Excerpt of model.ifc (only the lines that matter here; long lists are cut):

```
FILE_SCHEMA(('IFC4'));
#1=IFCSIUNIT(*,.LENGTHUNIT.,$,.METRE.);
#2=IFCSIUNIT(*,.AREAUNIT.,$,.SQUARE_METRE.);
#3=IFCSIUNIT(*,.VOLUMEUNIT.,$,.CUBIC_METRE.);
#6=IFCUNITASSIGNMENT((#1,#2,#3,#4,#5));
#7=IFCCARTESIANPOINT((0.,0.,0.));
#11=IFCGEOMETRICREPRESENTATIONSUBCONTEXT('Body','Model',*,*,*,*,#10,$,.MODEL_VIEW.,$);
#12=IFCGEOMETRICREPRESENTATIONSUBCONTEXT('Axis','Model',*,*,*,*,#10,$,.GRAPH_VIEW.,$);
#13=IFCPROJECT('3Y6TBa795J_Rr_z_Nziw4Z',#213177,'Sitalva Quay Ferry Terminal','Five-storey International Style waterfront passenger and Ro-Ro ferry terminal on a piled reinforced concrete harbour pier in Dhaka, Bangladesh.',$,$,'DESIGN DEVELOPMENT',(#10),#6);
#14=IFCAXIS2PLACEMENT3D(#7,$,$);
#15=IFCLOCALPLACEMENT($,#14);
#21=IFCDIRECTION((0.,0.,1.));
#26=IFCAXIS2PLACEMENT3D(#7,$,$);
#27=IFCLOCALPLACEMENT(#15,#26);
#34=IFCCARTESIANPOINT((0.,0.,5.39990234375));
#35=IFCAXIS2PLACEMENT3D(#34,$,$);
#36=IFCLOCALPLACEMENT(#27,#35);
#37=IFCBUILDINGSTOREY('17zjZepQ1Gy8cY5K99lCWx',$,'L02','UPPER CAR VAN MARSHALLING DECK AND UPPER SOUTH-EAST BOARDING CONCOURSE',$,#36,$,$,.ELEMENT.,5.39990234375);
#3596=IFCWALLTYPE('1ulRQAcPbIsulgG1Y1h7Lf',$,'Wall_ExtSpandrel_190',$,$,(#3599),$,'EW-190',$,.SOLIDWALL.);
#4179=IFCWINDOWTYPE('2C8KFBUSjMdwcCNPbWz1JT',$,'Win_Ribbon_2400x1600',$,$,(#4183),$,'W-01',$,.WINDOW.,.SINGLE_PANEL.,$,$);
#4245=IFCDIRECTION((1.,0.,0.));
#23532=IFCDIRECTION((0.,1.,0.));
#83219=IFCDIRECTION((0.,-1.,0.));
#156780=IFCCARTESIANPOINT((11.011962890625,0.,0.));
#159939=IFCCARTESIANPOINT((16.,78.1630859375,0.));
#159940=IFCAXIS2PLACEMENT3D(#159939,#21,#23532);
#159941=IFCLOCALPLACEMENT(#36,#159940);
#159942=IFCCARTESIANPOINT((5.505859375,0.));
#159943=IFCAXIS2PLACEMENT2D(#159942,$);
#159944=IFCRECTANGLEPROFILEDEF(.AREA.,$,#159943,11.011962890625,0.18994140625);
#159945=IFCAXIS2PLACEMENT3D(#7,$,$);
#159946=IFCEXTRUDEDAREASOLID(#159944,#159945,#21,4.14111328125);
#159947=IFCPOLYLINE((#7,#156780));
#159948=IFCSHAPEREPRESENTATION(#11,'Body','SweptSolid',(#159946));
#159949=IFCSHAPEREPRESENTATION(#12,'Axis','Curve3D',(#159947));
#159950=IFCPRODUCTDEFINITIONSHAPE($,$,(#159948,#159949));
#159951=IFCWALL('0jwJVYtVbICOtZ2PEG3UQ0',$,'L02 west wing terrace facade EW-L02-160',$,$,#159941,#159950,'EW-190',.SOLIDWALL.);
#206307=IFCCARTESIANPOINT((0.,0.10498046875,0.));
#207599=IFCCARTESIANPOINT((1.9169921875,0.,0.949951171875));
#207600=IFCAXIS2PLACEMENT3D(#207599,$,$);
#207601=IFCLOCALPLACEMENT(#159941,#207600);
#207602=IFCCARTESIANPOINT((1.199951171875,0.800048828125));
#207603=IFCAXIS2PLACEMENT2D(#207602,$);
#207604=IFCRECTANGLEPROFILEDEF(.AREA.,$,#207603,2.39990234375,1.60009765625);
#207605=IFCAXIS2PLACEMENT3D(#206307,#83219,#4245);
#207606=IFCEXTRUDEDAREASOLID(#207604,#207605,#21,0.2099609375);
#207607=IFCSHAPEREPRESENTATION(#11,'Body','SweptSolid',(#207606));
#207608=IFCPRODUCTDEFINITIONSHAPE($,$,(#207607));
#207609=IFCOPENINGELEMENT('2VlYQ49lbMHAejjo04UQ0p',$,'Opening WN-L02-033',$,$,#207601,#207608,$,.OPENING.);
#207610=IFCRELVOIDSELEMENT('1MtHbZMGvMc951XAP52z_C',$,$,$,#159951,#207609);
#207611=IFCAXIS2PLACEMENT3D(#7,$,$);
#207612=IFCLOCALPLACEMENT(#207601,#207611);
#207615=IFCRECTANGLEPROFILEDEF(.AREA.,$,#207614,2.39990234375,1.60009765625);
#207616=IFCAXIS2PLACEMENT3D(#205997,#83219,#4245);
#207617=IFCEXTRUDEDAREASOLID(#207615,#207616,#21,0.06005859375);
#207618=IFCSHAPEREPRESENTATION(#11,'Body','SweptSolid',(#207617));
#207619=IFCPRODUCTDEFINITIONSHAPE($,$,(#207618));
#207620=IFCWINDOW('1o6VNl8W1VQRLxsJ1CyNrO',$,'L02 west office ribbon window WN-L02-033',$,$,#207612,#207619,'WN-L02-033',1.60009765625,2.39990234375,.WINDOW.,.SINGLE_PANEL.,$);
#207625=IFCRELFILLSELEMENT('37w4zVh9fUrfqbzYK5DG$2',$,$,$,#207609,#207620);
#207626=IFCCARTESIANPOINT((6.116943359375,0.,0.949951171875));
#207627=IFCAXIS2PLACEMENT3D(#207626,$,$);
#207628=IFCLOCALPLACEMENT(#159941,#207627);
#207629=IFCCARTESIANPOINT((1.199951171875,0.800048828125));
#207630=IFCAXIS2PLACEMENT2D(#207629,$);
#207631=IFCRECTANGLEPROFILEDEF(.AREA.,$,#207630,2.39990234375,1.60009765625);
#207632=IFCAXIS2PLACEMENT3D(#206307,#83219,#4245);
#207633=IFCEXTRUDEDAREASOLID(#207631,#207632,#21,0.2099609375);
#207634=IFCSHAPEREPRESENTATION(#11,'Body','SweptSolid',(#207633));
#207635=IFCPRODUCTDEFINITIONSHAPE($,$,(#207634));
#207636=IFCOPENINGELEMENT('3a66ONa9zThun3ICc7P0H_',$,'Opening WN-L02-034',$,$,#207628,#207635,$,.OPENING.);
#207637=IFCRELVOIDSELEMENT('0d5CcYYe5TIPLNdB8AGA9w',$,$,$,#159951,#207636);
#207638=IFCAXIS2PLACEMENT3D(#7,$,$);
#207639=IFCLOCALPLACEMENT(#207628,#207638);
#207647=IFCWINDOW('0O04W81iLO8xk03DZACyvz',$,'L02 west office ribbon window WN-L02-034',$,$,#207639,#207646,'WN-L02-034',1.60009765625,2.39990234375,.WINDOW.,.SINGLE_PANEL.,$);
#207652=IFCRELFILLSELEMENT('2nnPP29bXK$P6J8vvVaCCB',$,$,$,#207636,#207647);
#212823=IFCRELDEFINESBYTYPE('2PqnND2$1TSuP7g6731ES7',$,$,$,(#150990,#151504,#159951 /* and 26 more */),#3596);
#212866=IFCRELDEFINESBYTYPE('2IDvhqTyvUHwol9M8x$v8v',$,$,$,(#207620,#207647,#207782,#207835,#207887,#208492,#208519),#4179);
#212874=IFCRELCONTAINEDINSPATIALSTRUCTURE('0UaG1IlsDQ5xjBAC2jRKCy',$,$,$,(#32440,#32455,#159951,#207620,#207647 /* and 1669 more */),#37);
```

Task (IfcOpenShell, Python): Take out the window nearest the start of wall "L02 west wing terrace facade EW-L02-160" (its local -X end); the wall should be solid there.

```python
import ifcopenshell
import ifcopenshell.api.feature
import ifcopenshell.api.root
import ifcopenshell.geom
import ifcopenshell.util.shape

model = ifcopenshell.open("model.ifc")
settings = ifcopenshell.geom.settings()


def volume(element):
    """Net volume in cubic metres, openings subtracted."""
    shape = ifcopenshell.geom.create_shape(settings, element)
    return ifcopenshell.util.shape.get_volume(shape.geometry)


window = model.by_id(207620)
opening = window.FillsVoids[0].RelatingOpeningElement
wall = opening.VoidsElements[0].RelatingBuildingElement
before = volume(wall)

ifcopenshell.api.root.remove_product(model, product=window)
ifcopenshell.api.feature.remove_feature(model, feature=opening)

after = volume(wall)

print(f"wall volume {before:.3f} -> {after:.3f} m3")

model.write("model_v2.ifc")
```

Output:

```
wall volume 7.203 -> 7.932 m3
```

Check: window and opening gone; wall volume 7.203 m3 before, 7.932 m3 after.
